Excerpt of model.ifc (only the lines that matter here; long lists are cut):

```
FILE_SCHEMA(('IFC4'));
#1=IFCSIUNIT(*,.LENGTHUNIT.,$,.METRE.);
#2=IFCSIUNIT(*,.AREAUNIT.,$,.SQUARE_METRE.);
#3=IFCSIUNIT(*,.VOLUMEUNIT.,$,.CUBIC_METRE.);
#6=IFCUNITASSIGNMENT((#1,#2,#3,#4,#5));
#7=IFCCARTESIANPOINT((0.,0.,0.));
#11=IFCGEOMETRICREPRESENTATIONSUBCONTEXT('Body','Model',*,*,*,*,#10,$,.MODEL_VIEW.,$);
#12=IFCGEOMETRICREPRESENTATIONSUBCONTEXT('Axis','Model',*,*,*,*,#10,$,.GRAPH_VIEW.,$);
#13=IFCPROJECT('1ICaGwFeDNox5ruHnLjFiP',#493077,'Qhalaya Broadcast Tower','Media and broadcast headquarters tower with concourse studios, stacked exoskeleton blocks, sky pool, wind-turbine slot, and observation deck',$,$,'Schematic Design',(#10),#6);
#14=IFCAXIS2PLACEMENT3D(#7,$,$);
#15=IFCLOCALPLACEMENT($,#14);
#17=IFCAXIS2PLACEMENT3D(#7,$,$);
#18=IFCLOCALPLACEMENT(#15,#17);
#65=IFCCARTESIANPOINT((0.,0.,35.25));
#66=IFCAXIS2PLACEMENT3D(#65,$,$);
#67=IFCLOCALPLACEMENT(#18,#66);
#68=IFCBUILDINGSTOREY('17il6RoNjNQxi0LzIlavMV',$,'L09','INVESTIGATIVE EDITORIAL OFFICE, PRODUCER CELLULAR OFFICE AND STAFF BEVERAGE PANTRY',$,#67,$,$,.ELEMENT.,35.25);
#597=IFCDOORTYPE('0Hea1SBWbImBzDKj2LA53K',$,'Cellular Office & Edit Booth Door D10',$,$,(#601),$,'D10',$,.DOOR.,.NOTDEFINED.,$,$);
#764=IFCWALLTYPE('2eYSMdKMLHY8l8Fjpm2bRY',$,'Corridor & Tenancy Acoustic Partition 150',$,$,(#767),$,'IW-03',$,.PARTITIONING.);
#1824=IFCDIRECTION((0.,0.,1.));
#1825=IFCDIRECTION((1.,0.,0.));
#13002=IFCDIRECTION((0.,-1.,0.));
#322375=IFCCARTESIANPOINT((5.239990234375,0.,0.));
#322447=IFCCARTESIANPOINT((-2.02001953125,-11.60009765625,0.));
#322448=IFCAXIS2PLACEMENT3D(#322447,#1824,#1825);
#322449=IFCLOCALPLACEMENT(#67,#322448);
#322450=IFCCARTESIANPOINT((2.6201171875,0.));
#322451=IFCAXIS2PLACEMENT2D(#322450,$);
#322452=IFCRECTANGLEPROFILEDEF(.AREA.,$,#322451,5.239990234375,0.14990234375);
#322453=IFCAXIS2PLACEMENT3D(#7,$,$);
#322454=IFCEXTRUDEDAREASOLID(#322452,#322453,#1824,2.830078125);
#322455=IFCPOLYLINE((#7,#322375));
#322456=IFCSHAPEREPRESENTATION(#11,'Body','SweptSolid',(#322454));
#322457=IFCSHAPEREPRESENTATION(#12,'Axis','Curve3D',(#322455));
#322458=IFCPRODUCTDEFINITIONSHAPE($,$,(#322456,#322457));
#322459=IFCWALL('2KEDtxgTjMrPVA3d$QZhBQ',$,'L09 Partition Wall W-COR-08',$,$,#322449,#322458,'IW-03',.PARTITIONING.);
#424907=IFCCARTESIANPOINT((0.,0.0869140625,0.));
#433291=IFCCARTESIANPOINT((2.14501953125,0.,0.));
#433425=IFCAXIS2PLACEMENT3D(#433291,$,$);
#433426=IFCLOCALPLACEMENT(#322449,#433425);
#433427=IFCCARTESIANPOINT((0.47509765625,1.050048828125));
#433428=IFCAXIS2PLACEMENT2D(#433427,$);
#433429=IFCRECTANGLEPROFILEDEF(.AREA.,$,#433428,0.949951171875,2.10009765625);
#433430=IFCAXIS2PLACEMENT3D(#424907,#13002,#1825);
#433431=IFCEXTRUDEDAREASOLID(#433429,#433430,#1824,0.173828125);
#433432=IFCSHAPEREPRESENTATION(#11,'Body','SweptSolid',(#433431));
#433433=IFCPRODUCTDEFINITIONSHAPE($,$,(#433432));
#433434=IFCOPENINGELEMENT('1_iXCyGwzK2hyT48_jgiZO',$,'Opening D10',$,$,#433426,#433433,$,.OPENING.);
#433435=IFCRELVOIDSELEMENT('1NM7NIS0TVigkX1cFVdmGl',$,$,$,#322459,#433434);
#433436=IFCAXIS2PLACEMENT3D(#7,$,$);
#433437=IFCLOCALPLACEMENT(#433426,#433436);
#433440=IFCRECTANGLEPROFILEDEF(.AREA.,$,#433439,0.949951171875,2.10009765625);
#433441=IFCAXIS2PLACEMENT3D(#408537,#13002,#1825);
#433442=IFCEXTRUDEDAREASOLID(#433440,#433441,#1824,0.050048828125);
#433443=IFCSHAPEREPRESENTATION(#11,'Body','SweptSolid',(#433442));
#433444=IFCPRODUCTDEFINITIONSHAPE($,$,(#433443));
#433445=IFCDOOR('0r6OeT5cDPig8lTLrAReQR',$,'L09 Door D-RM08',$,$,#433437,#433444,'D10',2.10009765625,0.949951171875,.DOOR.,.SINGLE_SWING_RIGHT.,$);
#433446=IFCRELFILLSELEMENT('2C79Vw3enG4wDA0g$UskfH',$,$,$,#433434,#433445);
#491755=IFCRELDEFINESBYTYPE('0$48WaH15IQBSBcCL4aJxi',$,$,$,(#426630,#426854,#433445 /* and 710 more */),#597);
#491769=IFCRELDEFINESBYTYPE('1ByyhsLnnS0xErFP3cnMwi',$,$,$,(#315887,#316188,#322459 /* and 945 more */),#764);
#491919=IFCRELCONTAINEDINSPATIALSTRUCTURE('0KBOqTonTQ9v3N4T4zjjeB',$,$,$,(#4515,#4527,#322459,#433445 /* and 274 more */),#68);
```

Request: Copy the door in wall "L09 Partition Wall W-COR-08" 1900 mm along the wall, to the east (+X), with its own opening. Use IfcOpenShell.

```python
import ifcopenshell
import ifcopenshell.api.feature
import ifcopenshell.api.geometry
import ifcopenshell.api.root
import ifcopenshell.geom
import ifcopenshell.util.element
import ifcopenshell.util.placement
import ifcopenshell.util.shape

model = ifcopenshell.open("model.ifc")
settings = ifcopenshell.geom.settings()


def volume(element):
    """Net volume in cubic metres, openings subtracted."""
    shape = ifcopenshell.geom.create_shape(settings, element)
    return ifcopenshell.util.shape.get_volume(shape.geometry)


door = model.by_guid("0r6OeT5cDPig8lTLrAReQR")
opening = door.FillsVoids[0].RelatingOpeningElement
wall = opening.VoidsElements[0].RelatingBuildingElement
before = volume(wall)
shift = ifcopenshell.util.placement.get_local_placement(wall.ObjectPlacement)[:3, 0] * 1.9

# copy_class copies the void relationship, type, container and properties, but no geometry.
new_opening = ifcopenshell.api.root.copy_class(model, product=opening)
new_opening.Representation = ifcopenshell.util.element.copy_deep(
    model, opening.Representation, exclude=["IfcGeometricRepresentationContext", "IfcRepresentationMap"]
)
new_door = ifcopenshell.api.root.copy_class(model, product=door)
new_door.Representation = ifcopenshell.util.element.copy_deep(
    model, door.Representation, exclude=["IfcGeometricRepresentationContext", "IfcRepresentationMap"]
)
new_door.Tag = None
ifcopenshell.api.feature.add_filling(model, opening=new_opening, element=new_door)

for old, new in ((opening, new_opening), (door, new_door)):
    matrix = ifcopenshell.util.placement.get_local_placement(old.ObjectPlacement)
    matrix[:3, 3] += shift
    ifcopenshell.api.geometry.edit_object_placement(model, product=new, matrix=matrix, is_si=False)

after = volume(wall)

print(f"wall volume {before:.3f} -> {after:.3f} m3")

model.write("model_edited.ifc")
```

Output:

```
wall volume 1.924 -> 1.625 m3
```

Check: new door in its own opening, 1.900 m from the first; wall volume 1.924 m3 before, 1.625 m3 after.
